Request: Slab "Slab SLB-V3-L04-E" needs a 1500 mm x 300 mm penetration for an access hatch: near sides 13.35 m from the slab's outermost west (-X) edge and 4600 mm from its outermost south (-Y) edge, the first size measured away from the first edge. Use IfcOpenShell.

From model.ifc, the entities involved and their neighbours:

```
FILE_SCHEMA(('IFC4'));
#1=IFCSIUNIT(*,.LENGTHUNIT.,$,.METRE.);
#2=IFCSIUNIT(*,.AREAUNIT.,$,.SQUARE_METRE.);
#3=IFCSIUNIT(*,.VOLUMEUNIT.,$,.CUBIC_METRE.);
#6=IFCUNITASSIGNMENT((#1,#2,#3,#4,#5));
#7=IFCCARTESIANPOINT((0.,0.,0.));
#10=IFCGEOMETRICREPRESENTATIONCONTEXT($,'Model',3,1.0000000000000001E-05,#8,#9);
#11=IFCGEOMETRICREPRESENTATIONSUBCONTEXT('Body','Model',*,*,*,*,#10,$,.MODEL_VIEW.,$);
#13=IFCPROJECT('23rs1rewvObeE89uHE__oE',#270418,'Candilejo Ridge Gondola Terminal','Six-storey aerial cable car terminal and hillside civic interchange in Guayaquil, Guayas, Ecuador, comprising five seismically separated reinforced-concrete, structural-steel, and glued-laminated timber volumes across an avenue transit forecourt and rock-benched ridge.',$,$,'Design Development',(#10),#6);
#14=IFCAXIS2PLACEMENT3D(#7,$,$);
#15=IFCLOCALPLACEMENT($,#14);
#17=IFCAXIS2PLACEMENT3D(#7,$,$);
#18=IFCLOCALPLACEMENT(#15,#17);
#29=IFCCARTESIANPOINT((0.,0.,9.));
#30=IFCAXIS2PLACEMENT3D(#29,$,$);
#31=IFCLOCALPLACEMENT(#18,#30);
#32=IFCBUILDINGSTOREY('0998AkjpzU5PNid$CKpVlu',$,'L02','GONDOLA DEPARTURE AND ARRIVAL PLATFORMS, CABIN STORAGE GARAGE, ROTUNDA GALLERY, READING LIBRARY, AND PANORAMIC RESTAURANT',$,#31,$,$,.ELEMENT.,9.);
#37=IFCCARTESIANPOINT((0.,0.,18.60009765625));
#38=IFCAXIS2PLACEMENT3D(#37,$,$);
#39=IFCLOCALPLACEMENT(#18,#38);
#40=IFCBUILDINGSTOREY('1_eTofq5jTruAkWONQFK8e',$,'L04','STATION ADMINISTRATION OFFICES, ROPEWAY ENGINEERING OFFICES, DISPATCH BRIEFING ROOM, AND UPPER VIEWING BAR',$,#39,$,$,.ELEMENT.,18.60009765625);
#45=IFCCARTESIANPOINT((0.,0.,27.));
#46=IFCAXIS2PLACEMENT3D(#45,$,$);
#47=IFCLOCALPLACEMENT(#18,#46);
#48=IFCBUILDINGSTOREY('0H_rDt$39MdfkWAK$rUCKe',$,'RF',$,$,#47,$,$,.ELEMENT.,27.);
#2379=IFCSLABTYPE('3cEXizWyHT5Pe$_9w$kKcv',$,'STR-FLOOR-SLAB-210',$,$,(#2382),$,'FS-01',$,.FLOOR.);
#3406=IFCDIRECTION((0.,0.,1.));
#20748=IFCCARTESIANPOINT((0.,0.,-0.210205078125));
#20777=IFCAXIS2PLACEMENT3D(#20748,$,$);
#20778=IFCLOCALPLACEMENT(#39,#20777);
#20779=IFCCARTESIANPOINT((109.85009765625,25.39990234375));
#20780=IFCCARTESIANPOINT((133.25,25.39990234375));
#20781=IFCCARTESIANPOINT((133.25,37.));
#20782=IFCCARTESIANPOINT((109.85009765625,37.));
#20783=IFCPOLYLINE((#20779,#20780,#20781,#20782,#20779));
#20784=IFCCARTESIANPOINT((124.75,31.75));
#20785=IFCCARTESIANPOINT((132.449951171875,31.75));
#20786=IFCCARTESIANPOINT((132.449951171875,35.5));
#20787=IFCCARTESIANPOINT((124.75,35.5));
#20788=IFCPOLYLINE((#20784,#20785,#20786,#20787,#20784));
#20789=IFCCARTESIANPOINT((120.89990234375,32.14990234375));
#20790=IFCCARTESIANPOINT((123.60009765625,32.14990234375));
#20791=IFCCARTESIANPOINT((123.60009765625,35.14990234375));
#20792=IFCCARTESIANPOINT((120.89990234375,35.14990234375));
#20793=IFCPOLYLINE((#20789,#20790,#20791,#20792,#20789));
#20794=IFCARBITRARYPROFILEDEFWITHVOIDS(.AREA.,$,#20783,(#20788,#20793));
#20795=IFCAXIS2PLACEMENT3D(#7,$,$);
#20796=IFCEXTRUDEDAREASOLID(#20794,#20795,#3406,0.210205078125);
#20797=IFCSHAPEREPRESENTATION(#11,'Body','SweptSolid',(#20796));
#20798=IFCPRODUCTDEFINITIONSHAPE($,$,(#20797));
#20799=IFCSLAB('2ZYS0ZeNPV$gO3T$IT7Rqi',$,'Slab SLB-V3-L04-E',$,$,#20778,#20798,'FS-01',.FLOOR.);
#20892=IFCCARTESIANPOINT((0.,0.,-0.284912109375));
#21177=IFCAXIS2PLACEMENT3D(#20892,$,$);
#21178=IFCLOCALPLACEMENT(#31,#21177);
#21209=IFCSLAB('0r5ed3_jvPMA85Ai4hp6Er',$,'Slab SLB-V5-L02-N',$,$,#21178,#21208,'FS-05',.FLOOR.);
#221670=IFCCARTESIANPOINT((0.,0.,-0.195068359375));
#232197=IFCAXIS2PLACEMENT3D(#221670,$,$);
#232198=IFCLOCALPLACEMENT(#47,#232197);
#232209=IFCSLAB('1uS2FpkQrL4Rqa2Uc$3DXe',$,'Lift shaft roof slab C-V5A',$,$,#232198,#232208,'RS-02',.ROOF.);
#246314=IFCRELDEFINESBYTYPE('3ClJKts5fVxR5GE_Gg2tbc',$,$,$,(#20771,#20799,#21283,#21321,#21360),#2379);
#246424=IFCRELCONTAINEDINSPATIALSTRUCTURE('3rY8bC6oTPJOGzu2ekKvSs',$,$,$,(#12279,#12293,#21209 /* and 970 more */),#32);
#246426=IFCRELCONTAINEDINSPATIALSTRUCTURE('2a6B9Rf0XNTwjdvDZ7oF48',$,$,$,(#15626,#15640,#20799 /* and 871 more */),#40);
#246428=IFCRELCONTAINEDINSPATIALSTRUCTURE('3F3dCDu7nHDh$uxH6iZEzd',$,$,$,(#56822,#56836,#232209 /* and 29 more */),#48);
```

```python
import numpy as np
import ifcopenshell
import ifcopenshell.api.feature
import ifcopenshell.api.geometry
import ifcopenshell.api.root
import ifcopenshell.geom
import ifcopenshell.util.placement
import ifcopenshell.util.representation
import ifcopenshell.util.shape
import ifcopenshell.util.unit

model = ifcopenshell.open("model.ifc")
unit_scale = ifcopenshell.util.unit.calculate_unit_scale(model)
settings = ifcopenshell.geom.settings()


def volume(element):
    """Net volume in cubic metres, openings subtracted."""
    shape = ifcopenshell.geom.create_shape(settings, element)
    return ifcopenshell.util.shape.get_volume(shape.geometry)


slab = model.by_guid("2ZYS0ZeNPV$gO3T$IT7Rqi")
before = volume(slab)

# Extent in the slab's own axes, in metres. The edges named are its -X and -Y sides.
slab_shape = ifcopenshell.geom.create_shape(settings, slab)
vertices = ifcopenshell.util.shape.get_vertices(slab_shape.geometry)
x_min, y_min, bottom = vertices.min(axis=0)
top = vertices[:, 2].max()

opening = ifcopenshell.api.root.create_entity(model, ifc_class="IfcOpeningElement", name="Access hatch opening", predefined_type="OPENING")
context = ifcopenshell.util.representation.get_context(model, "Model", "Body", "MODEL_VIEW")
width, depth = 1.5, 0.3
outline = [(0.0, 0.0), (width, 0.0), (width, depth), (0.0, depth), (0.0, 0.0)]
# Overshoot both faces by 50 mm so the cut is clean.
shape = ifcopenshell.api.geometry.add_slab_representation(
    model, context=context, depth=top - bottom + 0.1, polyline=outline
)
ifcopenshell.api.geometry.assign_representation(model, product=opening, representation=shape)

matrix = ifcopenshell.util.placement.get_local_placement(slab.ObjectPlacement)
matrix[:, 3] = matrix @ np.append(np.array([x_min + 13.35, y_min + 4.6, bottom - 0.05]) / unit_scale, 1.0)
ifcopenshell.api.geometry.edit_object_placement(model, product=opening, matrix=matrix, is_si=False)
ifcopenshell.api.feature.add_feature(model, feature=opening, element=slab)

after = volume(slab)

print(f"slab volume {before:.3f} -> {after:.3f} m3")

model.write("model_v2.ifc")
```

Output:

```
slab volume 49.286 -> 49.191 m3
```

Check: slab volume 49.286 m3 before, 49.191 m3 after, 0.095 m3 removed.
